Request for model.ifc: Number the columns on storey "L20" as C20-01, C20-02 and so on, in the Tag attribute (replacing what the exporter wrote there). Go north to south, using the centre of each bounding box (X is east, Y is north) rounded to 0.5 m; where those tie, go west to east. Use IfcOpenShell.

First a look at what the model holds.

```python
import ifcopenshell
import ifcopenshell.util.element
import ifcopenshell.util.placement

model = ifcopenshell.open("model.ifc")
print(model.schema)
storey = next(s for s in model.by_type("IfcBuildingStorey") if s.Name == "L20")
columns = [e for e in ifcopenshell.util.element.get_decomposition(storey) if e.is_a("IfcColumn")]
for e in sorted(columns, key=lambda e: e.id()):
    origin = ifcopenshell.util.placement.get_local_placement(e.ObjectPlacement)[:3, 3]
    print(e.id(), e.Tag, e.Name, origin.round(2) + 0.0, sep=" | ")
```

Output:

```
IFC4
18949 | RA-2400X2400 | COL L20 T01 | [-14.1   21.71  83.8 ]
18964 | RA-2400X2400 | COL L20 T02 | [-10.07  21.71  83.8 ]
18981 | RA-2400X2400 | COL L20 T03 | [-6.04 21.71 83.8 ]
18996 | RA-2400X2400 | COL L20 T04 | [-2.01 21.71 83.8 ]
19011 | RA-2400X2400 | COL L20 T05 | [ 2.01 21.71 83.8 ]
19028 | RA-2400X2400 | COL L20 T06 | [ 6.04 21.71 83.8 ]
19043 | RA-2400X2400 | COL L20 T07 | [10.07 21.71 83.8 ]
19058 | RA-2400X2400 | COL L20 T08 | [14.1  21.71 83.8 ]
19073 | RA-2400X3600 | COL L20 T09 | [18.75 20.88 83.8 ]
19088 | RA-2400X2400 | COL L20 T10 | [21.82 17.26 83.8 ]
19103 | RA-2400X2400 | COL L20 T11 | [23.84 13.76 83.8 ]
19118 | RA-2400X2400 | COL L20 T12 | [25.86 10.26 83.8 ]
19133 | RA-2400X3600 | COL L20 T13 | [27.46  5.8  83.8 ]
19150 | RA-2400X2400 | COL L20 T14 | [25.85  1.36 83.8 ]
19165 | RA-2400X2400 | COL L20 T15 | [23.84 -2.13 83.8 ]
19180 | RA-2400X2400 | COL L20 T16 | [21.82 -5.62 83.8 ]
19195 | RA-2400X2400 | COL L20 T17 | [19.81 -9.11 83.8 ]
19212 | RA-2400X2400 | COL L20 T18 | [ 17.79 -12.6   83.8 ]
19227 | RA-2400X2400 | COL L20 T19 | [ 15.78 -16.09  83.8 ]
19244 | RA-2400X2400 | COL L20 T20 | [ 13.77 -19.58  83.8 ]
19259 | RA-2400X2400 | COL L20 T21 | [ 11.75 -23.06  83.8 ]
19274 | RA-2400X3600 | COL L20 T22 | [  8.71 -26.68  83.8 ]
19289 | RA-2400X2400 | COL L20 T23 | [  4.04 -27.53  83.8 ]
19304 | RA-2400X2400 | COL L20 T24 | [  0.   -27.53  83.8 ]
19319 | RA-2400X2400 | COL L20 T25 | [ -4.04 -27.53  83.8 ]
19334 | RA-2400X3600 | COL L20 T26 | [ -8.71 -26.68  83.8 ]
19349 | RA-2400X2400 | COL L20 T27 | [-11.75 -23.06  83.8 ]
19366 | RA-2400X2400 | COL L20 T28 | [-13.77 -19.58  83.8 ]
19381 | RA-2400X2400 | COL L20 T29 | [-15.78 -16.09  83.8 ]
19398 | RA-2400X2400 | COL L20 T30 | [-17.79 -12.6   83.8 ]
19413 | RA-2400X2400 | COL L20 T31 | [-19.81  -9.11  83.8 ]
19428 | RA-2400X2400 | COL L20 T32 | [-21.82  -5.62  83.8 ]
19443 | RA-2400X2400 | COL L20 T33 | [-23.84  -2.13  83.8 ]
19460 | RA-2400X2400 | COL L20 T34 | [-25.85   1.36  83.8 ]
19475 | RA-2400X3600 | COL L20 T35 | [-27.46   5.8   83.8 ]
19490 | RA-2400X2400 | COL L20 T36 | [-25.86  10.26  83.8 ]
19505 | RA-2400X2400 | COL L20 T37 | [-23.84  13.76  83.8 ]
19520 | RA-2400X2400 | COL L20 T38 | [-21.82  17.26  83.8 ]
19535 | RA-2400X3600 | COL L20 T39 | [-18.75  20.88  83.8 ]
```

```python
import ifcopenshell
import ifcopenshell.geom
import ifcopenshell.util.element
import ifcopenshell.util.shape

model = ifcopenshell.open("model.ifc")
settings = ifcopenshell.geom.settings()
settings.set("use-world-coords", True)


def centre(element):
    shape = ifcopenshell.geom.create_shape(settings, element)
    return ifcopenshell.util.shape.get_bbox_centroid(shape.geometry)


storey = next(s for s in model.by_type("IfcBuildingStorey") if s.Name == "L20")
columns = [e for e in ifcopenshell.util.element.get_decomposition(storey) if e.is_a("IfcColumn")]

# Insertion points can sit at a corner or the storey origin, so sort by the geometry (in metres).
centres = {e: centre(e) for e in columns}
columns.sort(key=lambda e: (-round(centres[e][1] / 0.5), centres[e][0]))

for i, e in enumerate(columns, start=1):
    number = f"C20-{i:02d}"
    e.Tag = number
    print(e.id(), number)

model.write("model_v2.ifc")
```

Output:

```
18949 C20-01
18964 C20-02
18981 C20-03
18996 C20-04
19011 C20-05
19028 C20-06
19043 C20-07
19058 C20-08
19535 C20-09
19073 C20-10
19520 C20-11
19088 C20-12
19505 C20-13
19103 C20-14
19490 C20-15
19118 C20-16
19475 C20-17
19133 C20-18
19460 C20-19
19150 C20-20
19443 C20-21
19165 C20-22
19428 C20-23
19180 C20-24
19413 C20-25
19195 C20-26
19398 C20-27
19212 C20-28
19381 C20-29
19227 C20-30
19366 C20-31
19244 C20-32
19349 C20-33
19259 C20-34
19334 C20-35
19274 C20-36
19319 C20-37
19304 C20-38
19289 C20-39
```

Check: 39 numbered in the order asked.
